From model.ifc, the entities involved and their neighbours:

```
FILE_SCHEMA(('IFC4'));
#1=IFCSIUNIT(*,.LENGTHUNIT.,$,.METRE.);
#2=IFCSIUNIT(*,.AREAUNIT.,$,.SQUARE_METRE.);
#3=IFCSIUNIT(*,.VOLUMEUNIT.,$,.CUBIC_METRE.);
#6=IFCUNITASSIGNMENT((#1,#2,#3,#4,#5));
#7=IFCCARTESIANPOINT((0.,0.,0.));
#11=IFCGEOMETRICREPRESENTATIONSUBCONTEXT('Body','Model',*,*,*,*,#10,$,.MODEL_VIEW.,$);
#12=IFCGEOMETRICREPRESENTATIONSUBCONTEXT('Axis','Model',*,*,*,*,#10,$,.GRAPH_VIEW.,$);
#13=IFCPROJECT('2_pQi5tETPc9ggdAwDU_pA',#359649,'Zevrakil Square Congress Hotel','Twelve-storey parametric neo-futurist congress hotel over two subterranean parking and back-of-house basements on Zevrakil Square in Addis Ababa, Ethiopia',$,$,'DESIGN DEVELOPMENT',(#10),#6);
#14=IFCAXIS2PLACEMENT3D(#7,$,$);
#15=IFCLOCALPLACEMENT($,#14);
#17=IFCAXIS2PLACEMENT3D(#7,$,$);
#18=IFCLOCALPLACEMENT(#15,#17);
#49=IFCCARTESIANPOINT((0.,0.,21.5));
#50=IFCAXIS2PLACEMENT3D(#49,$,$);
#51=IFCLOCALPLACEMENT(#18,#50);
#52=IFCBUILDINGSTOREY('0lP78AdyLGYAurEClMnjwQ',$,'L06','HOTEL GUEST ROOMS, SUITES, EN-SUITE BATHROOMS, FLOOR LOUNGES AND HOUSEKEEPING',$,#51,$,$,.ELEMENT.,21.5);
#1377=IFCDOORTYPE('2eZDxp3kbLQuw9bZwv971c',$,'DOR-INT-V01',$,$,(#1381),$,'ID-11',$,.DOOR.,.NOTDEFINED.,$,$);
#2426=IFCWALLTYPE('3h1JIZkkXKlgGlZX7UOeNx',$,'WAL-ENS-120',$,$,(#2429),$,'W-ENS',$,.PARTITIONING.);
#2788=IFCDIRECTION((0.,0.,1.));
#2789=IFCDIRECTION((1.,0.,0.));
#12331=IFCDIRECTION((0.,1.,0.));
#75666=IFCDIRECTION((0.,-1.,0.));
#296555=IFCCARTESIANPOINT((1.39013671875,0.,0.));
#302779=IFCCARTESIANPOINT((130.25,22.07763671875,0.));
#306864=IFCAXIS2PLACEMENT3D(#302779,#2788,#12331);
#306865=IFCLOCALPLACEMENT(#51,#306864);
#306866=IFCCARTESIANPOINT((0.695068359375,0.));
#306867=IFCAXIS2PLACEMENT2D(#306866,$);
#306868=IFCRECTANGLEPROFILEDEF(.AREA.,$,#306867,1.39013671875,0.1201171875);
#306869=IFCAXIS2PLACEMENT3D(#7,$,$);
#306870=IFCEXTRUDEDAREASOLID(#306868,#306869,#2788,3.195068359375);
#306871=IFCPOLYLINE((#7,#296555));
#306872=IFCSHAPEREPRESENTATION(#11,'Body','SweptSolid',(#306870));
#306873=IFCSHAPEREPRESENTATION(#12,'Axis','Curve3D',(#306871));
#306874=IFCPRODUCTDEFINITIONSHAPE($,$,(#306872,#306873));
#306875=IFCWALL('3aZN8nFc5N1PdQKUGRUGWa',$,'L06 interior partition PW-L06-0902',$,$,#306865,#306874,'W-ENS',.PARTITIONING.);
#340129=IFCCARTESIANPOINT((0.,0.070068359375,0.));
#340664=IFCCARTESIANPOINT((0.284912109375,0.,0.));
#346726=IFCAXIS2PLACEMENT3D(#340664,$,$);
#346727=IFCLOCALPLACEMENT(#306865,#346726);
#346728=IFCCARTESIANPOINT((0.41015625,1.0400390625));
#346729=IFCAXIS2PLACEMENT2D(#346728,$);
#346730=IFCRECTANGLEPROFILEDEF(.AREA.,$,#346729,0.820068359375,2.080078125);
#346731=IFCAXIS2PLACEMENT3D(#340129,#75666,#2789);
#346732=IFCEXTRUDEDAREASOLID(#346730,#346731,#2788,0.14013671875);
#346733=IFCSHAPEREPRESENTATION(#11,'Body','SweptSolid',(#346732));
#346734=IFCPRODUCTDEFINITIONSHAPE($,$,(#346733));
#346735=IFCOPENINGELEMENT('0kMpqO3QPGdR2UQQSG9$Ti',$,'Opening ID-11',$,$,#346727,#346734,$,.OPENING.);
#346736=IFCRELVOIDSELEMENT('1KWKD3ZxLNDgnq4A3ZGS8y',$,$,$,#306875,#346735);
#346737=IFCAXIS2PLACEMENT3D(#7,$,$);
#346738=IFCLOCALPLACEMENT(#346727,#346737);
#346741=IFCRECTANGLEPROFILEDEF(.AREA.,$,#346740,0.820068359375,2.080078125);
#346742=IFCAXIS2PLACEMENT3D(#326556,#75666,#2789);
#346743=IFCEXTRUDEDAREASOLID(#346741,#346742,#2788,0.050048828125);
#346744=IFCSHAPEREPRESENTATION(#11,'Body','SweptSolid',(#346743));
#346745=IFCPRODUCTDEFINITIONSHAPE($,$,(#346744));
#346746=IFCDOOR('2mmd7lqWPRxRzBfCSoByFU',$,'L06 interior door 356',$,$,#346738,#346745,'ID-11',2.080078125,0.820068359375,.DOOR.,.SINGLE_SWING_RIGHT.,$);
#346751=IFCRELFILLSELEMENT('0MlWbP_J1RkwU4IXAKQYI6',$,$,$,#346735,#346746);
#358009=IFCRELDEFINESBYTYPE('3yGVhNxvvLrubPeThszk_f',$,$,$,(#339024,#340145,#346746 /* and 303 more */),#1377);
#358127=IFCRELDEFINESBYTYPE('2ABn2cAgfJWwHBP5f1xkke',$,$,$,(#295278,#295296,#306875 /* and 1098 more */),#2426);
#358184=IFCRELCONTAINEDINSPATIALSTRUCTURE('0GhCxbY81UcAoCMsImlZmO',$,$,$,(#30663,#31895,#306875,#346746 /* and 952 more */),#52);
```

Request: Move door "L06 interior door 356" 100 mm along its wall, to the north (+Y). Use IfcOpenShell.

```python
import ifcopenshell
import ifcopenshell.api.geometry
import ifcopenshell.util.placement

model = ifcopenshell.open("model.ifc")

door = model.by_guid("2mmd7lqWPRxRzBfCSoByFU")
opening = door.FillsVoids[0].RelatingOpeningElement
wall = opening.VoidsElements[0].RelatingBuildingElement

wall_matrix = ifcopenshell.util.placement.get_local_placement(wall.ObjectPlacement)
shift = wall_matrix[:3, 0] * 0.1
before = ifcopenshell.util.placement.get_local_placement(door.ObjectPlacement)[:3, 3].copy()

# The door is placed relative to its opening, so it follows when the opening moves.
matrix = ifcopenshell.util.placement.get_local_placement(opening.ObjectPlacement)
matrix[:3, 3] += shift
ifcopenshell.api.geometry.edit_object_placement(
    model, product=opening, matrix=matrix, is_si=False, should_transform_children=True
)

after = ifcopenshell.util.placement.get_local_placement(door.ObjectPlacement)[:3, 3]
print("door moved by", (after - before).round(3) + 0.0)

model.write("model_v2.ifc")
```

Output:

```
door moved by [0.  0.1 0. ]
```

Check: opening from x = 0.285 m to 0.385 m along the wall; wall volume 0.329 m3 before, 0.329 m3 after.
